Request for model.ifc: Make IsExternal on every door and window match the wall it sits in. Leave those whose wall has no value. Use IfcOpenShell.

First a look at what the model holds.

```python
import ifcopenshell
import ifcopenshell.util.element

model = ifcopenshell.open("model.ifc")
print(model.schema)
seen = {}
for e in model.by_type("IfcDoor") + model.by_type("IfcWindow"):
    if not e.FillsVoids:
        continue
    host = e.FillsVoids[0].RelatingOpeningElement.VoidsElements[0].RelatingBuildingElement
    own = ifcopenshell.util.element.get_pset(e, f"Pset_{e.is_a()[3:].removesuffix('StandardCase')}Common", "IsExternal")
    wall = ifcopenshell.util.element.get_pset(host, "Pset_WallCommon", "IsExternal")
    seen[e.is_a(), own, wall] = seen.get((e.is_a(), own, wall), 0) + 1
for (cls, own, wall), count in sorted(seen.items(), key=str):
    print(count, cls, "IsExternal:", own, "| host wall:", wall)
```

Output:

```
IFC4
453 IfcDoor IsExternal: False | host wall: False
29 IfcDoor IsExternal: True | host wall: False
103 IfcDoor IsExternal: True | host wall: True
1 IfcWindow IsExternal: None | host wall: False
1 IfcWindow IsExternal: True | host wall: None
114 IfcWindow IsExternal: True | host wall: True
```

```python
import ifcopenshell
import ifcopenshell.api.pset
import ifcopenshell.util.element

model = ifcopenshell.open("model.ifc")

count = 0
for ifc_class, pset_name in (("IfcDoor", "Pset_DoorCommon"), ("IfcWindow", "Pset_WindowCommon")):
    for e in model.by_type(ifc_class):
        if not e.FillsVoids:
            continue
        host = e.FillsVoids[0].RelatingOpeningElement.VoidsElements[0].RelatingBuildingElement
        external = ifcopenshell.util.element.get_pset(host, "Pset_WallCommon", "IsExternal")
        if external is None or ifcopenshell.util.element.get_pset(e, pset_name, "IsExternal") == external:
            continue
        pset = ifcopenshell.api.pset.add_pset(model, product=e, name=pset_name)
        ifcopenshell.api.pset.edit_pset(model, pset=pset, properties={"IsExternal": external})
        count += 1

print(count, "updated")

model.write("model_updated.ifc")
```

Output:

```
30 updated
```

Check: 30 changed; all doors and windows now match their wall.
